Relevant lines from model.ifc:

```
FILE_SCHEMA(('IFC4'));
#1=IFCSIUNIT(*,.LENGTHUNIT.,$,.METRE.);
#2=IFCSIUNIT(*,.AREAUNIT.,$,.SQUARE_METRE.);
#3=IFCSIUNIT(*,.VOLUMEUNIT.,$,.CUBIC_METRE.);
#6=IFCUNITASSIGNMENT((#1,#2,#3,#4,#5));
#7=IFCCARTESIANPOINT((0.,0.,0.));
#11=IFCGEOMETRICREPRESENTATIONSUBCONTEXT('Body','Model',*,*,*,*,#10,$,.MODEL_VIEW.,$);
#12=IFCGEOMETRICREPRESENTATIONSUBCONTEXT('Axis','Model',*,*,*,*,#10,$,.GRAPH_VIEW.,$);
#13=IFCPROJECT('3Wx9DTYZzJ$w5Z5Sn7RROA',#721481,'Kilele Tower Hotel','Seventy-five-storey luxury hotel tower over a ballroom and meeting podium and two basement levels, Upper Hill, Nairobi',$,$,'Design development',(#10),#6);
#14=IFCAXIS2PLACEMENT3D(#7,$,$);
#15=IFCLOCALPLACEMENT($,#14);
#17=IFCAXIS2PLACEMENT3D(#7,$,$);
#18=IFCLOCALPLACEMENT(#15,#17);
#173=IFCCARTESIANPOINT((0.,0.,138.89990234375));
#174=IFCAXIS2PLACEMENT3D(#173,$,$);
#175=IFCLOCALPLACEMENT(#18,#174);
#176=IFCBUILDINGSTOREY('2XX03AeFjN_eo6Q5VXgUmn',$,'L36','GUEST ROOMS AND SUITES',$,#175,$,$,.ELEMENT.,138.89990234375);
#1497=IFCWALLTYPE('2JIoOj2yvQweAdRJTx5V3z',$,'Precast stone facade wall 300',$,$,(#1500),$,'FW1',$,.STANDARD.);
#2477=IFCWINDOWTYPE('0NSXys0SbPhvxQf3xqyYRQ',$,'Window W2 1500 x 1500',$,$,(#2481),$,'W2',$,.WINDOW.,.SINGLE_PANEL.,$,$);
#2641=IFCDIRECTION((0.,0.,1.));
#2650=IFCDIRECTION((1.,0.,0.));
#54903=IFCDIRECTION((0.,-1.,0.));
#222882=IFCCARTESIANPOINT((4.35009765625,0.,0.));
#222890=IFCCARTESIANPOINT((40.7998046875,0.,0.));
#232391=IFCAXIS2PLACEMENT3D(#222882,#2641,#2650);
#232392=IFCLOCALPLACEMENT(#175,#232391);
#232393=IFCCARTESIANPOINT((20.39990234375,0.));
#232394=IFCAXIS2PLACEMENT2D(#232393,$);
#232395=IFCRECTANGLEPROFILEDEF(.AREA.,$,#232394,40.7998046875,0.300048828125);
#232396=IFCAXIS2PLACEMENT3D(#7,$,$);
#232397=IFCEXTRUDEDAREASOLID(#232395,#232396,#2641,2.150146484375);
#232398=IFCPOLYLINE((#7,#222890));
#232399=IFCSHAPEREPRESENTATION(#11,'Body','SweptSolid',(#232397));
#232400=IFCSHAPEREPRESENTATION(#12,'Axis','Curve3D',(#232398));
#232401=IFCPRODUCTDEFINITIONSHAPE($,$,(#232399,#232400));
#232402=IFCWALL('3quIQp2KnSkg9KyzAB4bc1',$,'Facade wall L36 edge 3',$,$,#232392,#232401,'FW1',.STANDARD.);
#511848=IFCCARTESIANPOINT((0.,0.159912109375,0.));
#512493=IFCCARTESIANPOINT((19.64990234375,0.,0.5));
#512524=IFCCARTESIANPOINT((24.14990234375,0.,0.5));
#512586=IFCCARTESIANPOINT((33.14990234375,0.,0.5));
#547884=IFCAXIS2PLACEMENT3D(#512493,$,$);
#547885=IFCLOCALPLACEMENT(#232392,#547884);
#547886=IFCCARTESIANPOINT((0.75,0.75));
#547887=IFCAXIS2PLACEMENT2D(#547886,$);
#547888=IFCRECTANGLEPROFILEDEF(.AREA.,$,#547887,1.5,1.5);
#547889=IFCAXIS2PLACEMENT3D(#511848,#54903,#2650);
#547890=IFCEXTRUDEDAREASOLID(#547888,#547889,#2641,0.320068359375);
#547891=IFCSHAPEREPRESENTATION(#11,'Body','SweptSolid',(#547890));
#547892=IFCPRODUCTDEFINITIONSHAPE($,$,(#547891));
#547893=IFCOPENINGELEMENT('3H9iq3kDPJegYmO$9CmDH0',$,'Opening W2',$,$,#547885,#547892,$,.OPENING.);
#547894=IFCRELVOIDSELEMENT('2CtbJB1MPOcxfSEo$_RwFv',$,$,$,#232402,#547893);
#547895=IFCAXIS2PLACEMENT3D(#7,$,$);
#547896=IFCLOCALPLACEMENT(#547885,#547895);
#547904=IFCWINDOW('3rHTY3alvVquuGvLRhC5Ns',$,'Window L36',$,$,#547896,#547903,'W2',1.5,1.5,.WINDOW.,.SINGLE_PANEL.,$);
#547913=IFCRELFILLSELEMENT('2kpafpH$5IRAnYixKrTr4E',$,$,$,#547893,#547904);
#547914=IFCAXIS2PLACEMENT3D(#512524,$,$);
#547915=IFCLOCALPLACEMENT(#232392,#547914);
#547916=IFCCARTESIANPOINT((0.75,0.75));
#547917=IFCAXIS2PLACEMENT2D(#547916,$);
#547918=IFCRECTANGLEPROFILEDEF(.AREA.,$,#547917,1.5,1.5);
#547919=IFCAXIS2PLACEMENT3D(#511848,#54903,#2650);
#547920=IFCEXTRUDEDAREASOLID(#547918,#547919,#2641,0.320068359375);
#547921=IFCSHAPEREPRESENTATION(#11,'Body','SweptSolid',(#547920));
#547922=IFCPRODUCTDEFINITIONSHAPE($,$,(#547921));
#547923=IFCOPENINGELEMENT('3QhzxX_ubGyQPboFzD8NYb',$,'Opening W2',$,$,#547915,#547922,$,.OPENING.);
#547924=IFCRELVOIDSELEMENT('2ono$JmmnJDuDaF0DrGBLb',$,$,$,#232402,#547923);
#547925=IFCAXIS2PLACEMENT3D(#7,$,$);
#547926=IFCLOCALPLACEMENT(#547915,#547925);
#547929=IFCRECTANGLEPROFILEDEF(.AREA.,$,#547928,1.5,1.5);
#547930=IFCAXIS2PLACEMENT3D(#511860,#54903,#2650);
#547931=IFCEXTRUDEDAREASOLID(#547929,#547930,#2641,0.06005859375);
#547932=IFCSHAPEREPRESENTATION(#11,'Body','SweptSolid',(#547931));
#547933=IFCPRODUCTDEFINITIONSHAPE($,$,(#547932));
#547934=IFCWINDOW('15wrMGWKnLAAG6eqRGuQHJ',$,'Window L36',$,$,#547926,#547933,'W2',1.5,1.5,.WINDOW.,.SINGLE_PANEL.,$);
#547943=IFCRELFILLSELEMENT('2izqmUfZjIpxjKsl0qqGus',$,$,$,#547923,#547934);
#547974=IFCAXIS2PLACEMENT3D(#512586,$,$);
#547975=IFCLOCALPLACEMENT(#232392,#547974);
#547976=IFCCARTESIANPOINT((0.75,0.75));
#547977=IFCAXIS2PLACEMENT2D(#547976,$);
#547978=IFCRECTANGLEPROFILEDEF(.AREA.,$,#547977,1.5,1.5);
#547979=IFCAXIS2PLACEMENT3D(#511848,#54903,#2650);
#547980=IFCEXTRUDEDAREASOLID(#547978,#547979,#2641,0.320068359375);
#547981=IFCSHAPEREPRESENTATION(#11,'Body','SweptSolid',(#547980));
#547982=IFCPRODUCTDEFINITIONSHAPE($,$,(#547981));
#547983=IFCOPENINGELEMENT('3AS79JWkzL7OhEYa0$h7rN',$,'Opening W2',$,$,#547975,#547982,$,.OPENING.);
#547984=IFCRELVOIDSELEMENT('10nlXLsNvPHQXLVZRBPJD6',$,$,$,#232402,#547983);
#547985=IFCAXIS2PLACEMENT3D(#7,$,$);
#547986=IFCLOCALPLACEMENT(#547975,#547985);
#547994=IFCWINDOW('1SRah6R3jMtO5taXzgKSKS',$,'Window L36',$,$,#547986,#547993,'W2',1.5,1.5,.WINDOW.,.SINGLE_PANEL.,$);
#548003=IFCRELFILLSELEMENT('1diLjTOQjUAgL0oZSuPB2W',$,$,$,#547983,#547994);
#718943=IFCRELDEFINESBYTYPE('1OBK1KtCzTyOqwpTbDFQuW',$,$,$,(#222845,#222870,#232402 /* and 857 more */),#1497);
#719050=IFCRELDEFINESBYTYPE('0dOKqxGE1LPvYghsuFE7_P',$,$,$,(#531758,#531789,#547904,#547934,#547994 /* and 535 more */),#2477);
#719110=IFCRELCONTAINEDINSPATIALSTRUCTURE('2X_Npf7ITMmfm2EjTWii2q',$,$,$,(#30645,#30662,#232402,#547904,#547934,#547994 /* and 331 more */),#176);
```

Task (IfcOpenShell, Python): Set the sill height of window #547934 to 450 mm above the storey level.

```python
import numpy as np
import ifcopenshell
import ifcopenshell.api.geometry
import ifcopenshell.geom
import ifcopenshell.util.element
import ifcopenshell.util.placement
import ifcopenshell.util.shape
import ifcopenshell.util.unit

model = ifcopenshell.open("model.ifc")
unit_scale = ifcopenshell.util.unit.calculate_unit_scale(model)

window = model.by_guid("15wrMGWKnLAAG6eqRGuQHJ")
opening = window.FillsVoids[0].RelatingOpeningElement
storey = ifcopenshell.util.element.get_container(window, ifc_class="IfcBuildingStorey")
level = ifcopenshell.util.placement.get_local_placement(storey.ObjectPlacement)[2, 3]

# The opening's origin need not be at the sill, so measure its lowest point.
shape = ifcopenshell.geom.create_shape(ifcopenshell.geom.settings(), opening)
bottom = ifcopenshell.util.shape.get_shape_bottom_elevation(shape, shape.geometry) / unit_scale
dz = level + 0.45 / unit_scale - bottom

shift = np.array([0.0, 0.0, dz])
# The window is placed relative to its opening, so it follows when the opening moves.
matrix = ifcopenshell.util.placement.get_local_placement(opening.ObjectPlacement)
matrix[:3, 3] += shift
ifcopenshell.api.geometry.edit_object_placement(
    model, product=opening, matrix=matrix, is_si=False, should_transform_children=True
)

print(f"moved by {dz * unit_scale:+.3f} m")

model.write("model_updated.ifc")
```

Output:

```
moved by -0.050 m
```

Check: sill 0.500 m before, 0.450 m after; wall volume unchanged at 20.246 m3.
